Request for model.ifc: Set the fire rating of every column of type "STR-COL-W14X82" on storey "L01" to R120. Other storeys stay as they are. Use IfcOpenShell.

First a look at what the model holds.

```python
import ifcopenshell
import ifcopenshell.util.element

model = ifcopenshell.open("model.ifc")
print(model.schema)
storey = next(s for s in model.by_type("IfcBuildingStorey") if s.Name == "L01")
columns = [e for e in ifcopenshell.util.element.get_decomposition(storey) if e.is_a("IfcColumn")]
seen = {}
for e in columns:
    element_type = ifcopenshell.util.element.get_type(e)
    key = (element_type.Name if element_type != e and element_type else None, ifcopenshell.util.element.get_pset(e, "Pset_ColumnCommon", "FireRating"))
    seen[key] = seen.get(key, 0) + 1
for (name, value), count in sorted(seen.items(), key=str):
    print(count, "x", name, "|", value)
```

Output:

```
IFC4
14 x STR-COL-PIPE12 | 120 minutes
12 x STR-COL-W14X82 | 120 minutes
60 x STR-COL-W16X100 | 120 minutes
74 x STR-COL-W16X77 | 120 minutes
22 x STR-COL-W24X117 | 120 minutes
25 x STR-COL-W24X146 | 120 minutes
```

```python
import ifcopenshell
import ifcopenshell.api.pset
import ifcopenshell.util.element

model = ifcopenshell.open("model.ifc")

storey = next(s for s in model.by_type("IfcBuildingStorey") if s.Name == "L01")
columns = [e for e in ifcopenshell.util.element.get_decomposition(storey) if e.is_a("IfcColumn")]

count = 0
for e in columns:
    element_type = ifcopenshell.util.element.get_type(e)
    if element_type in (None, e) or element_type.Name != "STR-COL-W14X82":
        continue
    # add_pset returns the element's existing set when there is one.
    pset = ifcopenshell.api.pset.add_pset(model, product=e, name="Pset_ColumnCommon")
    ifcopenshell.api.pset.edit_pset(model, pset=pset, properties={"FireRating": "R120"})
    count += 1

print(count, "columns updated")

model.write("model_edited.ifc")
```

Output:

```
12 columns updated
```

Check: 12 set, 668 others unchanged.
